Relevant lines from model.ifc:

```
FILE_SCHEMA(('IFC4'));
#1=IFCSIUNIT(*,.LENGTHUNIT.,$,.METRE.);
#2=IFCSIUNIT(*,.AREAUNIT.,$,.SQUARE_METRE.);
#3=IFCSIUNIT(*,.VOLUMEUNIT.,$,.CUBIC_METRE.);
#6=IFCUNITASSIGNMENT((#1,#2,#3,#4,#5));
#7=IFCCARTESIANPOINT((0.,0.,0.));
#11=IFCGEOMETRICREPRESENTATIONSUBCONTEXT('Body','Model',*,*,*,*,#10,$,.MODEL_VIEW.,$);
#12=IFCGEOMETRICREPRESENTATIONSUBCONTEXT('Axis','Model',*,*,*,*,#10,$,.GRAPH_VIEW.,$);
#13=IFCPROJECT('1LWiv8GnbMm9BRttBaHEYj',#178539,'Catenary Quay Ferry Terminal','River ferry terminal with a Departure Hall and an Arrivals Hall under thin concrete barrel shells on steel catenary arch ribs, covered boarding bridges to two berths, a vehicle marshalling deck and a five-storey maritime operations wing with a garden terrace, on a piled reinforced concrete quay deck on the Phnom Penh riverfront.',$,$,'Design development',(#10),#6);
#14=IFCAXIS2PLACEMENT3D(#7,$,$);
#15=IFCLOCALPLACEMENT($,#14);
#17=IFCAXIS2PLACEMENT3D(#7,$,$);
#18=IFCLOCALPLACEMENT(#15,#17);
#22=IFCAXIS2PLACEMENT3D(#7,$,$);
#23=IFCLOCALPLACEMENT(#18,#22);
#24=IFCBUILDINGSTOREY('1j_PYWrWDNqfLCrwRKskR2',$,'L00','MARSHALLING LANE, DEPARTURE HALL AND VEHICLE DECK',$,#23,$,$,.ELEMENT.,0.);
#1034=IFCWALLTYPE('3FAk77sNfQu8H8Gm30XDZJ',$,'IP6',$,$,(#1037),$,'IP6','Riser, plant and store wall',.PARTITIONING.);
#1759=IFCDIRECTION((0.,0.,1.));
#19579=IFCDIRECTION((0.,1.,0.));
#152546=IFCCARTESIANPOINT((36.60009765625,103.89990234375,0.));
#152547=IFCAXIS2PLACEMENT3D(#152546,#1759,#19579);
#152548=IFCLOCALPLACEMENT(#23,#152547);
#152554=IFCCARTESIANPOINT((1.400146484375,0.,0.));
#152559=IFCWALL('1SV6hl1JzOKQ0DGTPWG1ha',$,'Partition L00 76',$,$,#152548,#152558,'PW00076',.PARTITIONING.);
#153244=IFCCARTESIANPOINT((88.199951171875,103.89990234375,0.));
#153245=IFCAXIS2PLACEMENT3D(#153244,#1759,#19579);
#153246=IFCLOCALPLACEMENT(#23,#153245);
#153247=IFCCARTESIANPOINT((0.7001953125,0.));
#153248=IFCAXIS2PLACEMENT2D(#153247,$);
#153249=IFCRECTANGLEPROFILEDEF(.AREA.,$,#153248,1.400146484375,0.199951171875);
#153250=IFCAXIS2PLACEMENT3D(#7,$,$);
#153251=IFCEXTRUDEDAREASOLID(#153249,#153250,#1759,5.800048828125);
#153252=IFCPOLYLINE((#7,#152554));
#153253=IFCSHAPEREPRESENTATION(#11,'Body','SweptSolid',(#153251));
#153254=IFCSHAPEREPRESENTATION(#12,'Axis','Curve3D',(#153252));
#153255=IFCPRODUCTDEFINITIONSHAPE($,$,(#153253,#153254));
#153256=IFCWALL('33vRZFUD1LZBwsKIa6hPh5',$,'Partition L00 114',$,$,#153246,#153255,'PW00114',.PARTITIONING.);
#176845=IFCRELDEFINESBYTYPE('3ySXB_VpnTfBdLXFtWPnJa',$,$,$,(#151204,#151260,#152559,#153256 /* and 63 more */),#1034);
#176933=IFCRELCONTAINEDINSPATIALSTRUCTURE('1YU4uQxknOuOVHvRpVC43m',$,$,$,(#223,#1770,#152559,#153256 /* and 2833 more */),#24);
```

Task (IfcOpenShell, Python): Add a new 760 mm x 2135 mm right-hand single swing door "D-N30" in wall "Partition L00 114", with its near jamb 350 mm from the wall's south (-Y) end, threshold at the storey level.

```python
import numpy as np
import ifcopenshell
import ifcopenshell.api.feature
import ifcopenshell.api.geometry
import ifcopenshell.api.root
import ifcopenshell.api.spatial
import ifcopenshell.geom
import ifcopenshell.util.element
import ifcopenshell.util.placement
import ifcopenshell.util.representation
import ifcopenshell.util.shape
import ifcopenshell.util.unit

model = ifcopenshell.open("model.ifc")
unit_scale = ifcopenshell.util.unit.calculate_unit_scale(model)
settings = ifcopenshell.geom.settings()


def volume(element):
    """Net volume in cubic metres, openings subtracted."""
    shape = ifcopenshell.geom.create_shape(settings, element)
    return ifcopenshell.util.shape.get_volume(shape.geometry)


wall = model.by_guid("33vRZFUD1LZBwsKIa6hPh5")
storey = ifcopenshell.util.element.get_container(wall, ifc_class="IfcBuildingStorey")
context = ifcopenshell.util.representation.get_context(model, "Model", "Body", "MODEL_VIEW")
before = volume(wall)

width, height, from_end, sill = 0.76, 2.135, 0.35, 0.0  # metres

# The wall runs along its own X axis, and the end named is its -X end.
wall_shape = ifcopenshell.geom.create_shape(settings, wall)
x, y, z = ifcopenshell.util.shape.get_vertices(wall_shape.geometry).T
start = x.min() + from_end
face, thickness = float(y.min()), float(y.max() - y.min())
wall_matrix = ifcopenshell.util.placement.get_local_placement(wall.ObjectPlacement)
level = ifcopenshell.util.placement.get_local_placement(storey.ObjectPlacement)[2, 3]


def in_wall(x, y):
    """Placement at x, y metres in the wall's axes, at sill height."""
    matrix = wall_matrix.copy()
    matrix[:, 3] = wall_matrix @ np.array([x / unit_scale, y / unit_scale, 0.0, 1.0])
    matrix[2, 3] = level + sill / unit_scale
    return matrix


# Opening: a box that overshoots both wall faces by 50 mm.
opening = ifcopenshell.api.root.create_entity(model, ifc_class="IfcOpeningElement", predefined_type="OPENING")
box = ifcopenshell.api.geometry.add_wall_representation(
    model, context=context, length=width, height=height, thickness=thickness + 0.1
)
ifcopenshell.api.geometry.assign_representation(model, product=opening, representation=box)
ifcopenshell.api.geometry.edit_object_placement(model, product=opening, matrix=in_wall(start, face - 0.05), is_si=False)
ifcopenshell.api.feature.add_feature(model, feature=opening, element=wall)

door = ifcopenshell.api.root.create_entity(model, ifc_class="IfcDoor", name="D-N30", predefined_type="DOOR")
door.OverallWidth, door.OverallHeight = width / unit_scale, height / unit_scale
door.OperationType = "SINGLE_SWING_RIGHT"
body = ifcopenshell.api.geometry.add_door_representation(
    model,
    context=context,
    overall_width=door.OverallWidth,
    overall_height=door.OverallHeight,
    operation_type="SINGLE_SWING_RIGHT",
    lining_properties={"LiningDepth": thickness / unit_scale, "ThresholdDepth": thickness / unit_scale},
)
ifcopenshell.api.geometry.assign_representation(model, product=door, representation=body)
ifcopenshell.api.spatial.assign_container(model, products=[door], relating_structure=storey)
ifcopenshell.api.feature.add_filling(model, opening=opening, element=door)

# The lining spans the wall, so the door starts at the wall face.
ifcopenshell.api.geometry.edit_object_placement(model, product=door, matrix=in_wall(start, face), is_si=False)

after = volume(wall)

print(f"wall volume {before:.3f} -> {after:.3f} m3")

model.write("model_v2.ifc")
```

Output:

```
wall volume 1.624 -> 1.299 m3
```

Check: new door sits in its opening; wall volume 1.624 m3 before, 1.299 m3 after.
